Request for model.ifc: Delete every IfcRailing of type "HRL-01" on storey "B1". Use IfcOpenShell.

First a look at what the model holds.

```python
import ifcopenshell
import ifcopenshell.util.element

model = ifcopenshell.open("model.ifc")
print(model.schema)
storey = next(s for s in model.by_type("IfcBuildingStorey") if s.Name == "B1")
railings = [e for e in ifcopenshell.util.element.get_decomposition(storey) if e.is_a("IfcRailing")]
seen = {}
for e in railings:
    element_type = ifcopenshell.util.element.get_type(e)
    name = element_type.Name if element_type not in (None, e) else None
    seen[name] = seen.get(name, 0) + 1
for name, count in sorted(seen.items(), key=str):
    print(count, "x", name)
```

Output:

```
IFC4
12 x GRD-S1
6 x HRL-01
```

```python
import ifcopenshell
import ifcopenshell.api.root
import ifcopenshell.util.element

model = ifcopenshell.open("model.ifc")

storey = next(s for s in model.by_type("IfcBuildingStorey") if s.Name == "B1")
railings = [e for e in ifcopenshell.util.element.get_decomposition(storey) if e.is_a("IfcRailing")]
targets = [e for e in railings if (t := ifcopenshell.util.element.get_type(e)) not in (None, e) and t.Name == "HRL-01"]

for e in targets:
    ifcopenshell.api.root.remove_product(model, product=e)
print(len(targets), "removed")

model.write("model-out.ifc")
```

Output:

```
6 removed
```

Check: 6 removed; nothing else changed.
